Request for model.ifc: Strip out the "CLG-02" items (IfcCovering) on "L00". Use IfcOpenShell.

First a look at what the model holds.

```python
import ifcopenshell
import ifcopenshell.util.element

model = ifcopenshell.open("model.ifc")
print(model.schema)
storey = next(s for s in model.by_type("IfcBuildingStorey") if s.Name == "L00")
coverings = [e for e in ifcopenshell.util.element.get_decomposition(storey) if e.is_a("IfcCovering")]
seen = {}
for e in coverings:
    element_type = ifcopenshell.util.element.get_type(e)
    name = element_type.Name if element_type not in (None, e) else None
    seen[name] = seen.get(name, 0) + 1
for name, count in sorted(seen.items(), key=str):
    print(count, "x", name)
```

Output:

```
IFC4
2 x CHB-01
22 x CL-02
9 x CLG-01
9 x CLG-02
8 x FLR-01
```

```python
import ifcopenshell
import ifcopenshell.api.root
import ifcopenshell.util.element

model = ifcopenshell.open("model.ifc")

storey = next(s for s in model.by_type("IfcBuildingStorey") if s.Name == "L00")
coverings = [e for e in ifcopenshell.util.element.get_decomposition(storey) if e.is_a("IfcCovering")]
targets = [e for e in coverings if (t := ifcopenshell.util.element.get_type(e)) not in (None, e) and t.Name == "CLG-02"]

for e in targets:
    ifcopenshell.api.root.remove_product(model, product=e)
print(len(targets), "removed")

model.write("model-out.ifc")
```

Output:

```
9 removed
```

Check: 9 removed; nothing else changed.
